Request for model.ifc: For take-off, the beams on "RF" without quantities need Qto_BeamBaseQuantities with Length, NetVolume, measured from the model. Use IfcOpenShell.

First a look at what the model holds.

```python
import ifcopenshell
import ifcopenshell.util.element
import ifcopenshell.util.unit

model = ifcopenshell.open("model.ifc")
print(model.schema)
for unit_type in ("LENGTHUNIT", "AREAUNIT", "VOLUMEUNIT"):
    print(unit_type, ifcopenshell.util.unit.calculate_unit_scale(model, unit_type))
storey = next(s for s in model.by_type("IfcBuildingStorey") if s.Name == "RF")
beams = [e for e in ifcopenshell.util.element.get_decomposition(storey) if e.is_a("IfcBeam")]
for e in sorted(beams, key=lambda e: e.id()):
    print(e.id(), e.is_a(), e.Name, list(ifcopenshell.util.element.get_psets(e, qtos_only=True)), sep=" | ")
```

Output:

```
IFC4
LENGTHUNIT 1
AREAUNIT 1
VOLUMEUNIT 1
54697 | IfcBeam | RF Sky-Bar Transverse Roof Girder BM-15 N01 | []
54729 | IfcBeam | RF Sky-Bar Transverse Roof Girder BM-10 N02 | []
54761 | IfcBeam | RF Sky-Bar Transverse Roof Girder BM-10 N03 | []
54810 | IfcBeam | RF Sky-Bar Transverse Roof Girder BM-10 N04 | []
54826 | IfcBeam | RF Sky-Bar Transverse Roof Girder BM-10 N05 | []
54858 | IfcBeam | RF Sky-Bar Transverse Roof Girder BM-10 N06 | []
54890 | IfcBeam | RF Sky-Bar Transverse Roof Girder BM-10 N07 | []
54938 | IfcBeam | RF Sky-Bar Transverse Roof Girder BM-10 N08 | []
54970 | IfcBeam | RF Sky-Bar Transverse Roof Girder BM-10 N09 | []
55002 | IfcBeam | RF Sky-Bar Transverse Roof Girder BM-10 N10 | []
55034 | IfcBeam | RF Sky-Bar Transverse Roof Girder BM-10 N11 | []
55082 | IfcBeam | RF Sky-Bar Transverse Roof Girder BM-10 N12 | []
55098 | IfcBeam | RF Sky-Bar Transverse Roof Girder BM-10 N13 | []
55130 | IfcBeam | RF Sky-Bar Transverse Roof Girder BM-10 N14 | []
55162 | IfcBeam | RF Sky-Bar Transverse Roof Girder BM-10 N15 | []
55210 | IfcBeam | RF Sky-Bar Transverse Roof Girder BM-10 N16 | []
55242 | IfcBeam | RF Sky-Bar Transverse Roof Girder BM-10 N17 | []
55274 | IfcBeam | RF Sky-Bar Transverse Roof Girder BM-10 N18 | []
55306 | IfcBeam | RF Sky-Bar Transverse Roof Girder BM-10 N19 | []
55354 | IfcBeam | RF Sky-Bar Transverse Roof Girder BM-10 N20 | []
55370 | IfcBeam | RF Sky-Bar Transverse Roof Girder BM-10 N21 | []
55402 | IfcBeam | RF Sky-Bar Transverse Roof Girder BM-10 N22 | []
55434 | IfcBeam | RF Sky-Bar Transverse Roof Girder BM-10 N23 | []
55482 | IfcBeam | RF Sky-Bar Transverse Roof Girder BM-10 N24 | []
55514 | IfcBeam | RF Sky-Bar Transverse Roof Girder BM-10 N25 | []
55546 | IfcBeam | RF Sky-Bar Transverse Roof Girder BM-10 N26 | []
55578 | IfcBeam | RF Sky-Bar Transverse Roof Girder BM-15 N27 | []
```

```python
import ifcopenshell
import ifcopenshell.api.pset
import ifcopenshell.geom
import ifcopenshell.util.element
import ifcopenshell.util.shape
import ifcopenshell.util.unit

model = ifcopenshell.open("model.ifc")
unit_scale = ifcopenshell.util.unit.calculate_unit_scale(model)
volume_scale = ifcopenshell.util.unit.calculate_unit_scale(model, "VOLUMEUNIT")
settings = ifcopenshell.geom.settings()

storey = next(s for s in model.by_type("IfcBuildingStorey") if s.Name == "RF")
beams = [e for e in ifcopenshell.util.element.get_decomposition(storey) if e.is_a("IfcBeam")]

for e in sorted(beams, key=lambda e: e.id()):
    if ifcopenshell.util.element.get_psets(e, qtos_only=True, should_inherit=False):
        continue
    # Geometry comes back in metres, in the element's own axes.
    shape = ifcopenshell.geom.create_shape(settings, e)
    values = {
        "Length": ifcopenshell.util.shape.get_max_xyz(shape.geometry) / unit_scale,
        "NetVolume": ifcopenshell.util.shape.get_volume(shape.geometry) / volume_scale,
    }
    qto = ifcopenshell.api.pset.add_qto(model, product=e, name="Qto_BeamBaseQuantities")
    ifcopenshell.api.pset.edit_qto(model, qto=qto, properties=values)
    print(e.id(), {k: round(v, 3) for k, v in values.items()})

model.write("model_edited.ifc")
```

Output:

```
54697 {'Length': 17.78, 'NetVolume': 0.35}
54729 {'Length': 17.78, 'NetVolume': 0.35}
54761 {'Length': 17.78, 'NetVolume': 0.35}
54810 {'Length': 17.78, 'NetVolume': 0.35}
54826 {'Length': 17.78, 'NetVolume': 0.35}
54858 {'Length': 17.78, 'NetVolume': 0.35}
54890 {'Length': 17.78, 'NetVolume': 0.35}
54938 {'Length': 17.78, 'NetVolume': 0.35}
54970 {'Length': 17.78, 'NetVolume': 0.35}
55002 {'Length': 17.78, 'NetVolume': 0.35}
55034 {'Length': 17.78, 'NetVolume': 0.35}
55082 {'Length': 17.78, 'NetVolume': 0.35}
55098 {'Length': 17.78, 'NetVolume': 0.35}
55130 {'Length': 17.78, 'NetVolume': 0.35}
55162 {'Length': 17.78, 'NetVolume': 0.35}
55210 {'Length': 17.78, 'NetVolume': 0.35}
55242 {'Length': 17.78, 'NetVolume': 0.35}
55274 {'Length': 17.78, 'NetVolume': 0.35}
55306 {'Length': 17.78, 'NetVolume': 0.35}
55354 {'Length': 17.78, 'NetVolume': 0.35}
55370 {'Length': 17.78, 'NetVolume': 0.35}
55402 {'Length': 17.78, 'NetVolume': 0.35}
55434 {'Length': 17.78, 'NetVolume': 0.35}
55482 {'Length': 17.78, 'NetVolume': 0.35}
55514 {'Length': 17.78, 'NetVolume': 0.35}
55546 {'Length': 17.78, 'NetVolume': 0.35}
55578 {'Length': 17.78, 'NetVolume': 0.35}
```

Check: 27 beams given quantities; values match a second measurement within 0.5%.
